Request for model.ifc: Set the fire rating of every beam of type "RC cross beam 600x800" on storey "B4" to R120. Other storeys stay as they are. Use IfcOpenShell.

First a look at what the model holds.

```python
import ifcopenshell
import ifcopenshell.util.element

model = ifcopenshell.open("model.ifc")
print(model.schema)
storey = next(s for s in model.by_type("IfcBuildingStorey") if s.Name == "B4")
beams = [e for e in ifcopenshell.util.element.get_decomposition(storey) if e.is_a("IfcBeam")]
seen = {}
for e in beams:
    element_type = ifcopenshell.util.element.get_type(e)
    key = (element_type.Name if element_type != e and element_type else None, ifcopenshell.util.element.get_pset(e, "Pset_BeamCommon", "FireRating"))
    seen[key] = seen.get(key, 0) + 1
for (name, value), count in sorted(seen.items(), key=str):
    print(count, "x", name, "|", value)
```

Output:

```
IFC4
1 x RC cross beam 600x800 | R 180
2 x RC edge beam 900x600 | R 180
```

```python
import ifcopenshell
import ifcopenshell.api.pset
import ifcopenshell.util.element

model = ifcopenshell.open("model.ifc")

storey = next(s for s in model.by_type("IfcBuildingStorey") if s.Name == "B4")
beams = [e for e in ifcopenshell.util.element.get_decomposition(storey) if e.is_a("IfcBeam")]

count = 0
for e in beams:
    element_type = ifcopenshell.util.element.get_type(e)
    if element_type in (None, e) or element_type.Name != "RC cross beam 600x800":
        continue
    # add_pset returns the element's existing set when there is one.
    pset = ifcopenshell.api.pset.add_pset(model, product=e, name="Pset_BeamCommon")
    ifcopenshell.api.pset.edit_pset(model, pset=pset, properties={"FireRating": "R120"})
    count += 1

print(count, "beams updated")

model.write("model_rev.ifc")
```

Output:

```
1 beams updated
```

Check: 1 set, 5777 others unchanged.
